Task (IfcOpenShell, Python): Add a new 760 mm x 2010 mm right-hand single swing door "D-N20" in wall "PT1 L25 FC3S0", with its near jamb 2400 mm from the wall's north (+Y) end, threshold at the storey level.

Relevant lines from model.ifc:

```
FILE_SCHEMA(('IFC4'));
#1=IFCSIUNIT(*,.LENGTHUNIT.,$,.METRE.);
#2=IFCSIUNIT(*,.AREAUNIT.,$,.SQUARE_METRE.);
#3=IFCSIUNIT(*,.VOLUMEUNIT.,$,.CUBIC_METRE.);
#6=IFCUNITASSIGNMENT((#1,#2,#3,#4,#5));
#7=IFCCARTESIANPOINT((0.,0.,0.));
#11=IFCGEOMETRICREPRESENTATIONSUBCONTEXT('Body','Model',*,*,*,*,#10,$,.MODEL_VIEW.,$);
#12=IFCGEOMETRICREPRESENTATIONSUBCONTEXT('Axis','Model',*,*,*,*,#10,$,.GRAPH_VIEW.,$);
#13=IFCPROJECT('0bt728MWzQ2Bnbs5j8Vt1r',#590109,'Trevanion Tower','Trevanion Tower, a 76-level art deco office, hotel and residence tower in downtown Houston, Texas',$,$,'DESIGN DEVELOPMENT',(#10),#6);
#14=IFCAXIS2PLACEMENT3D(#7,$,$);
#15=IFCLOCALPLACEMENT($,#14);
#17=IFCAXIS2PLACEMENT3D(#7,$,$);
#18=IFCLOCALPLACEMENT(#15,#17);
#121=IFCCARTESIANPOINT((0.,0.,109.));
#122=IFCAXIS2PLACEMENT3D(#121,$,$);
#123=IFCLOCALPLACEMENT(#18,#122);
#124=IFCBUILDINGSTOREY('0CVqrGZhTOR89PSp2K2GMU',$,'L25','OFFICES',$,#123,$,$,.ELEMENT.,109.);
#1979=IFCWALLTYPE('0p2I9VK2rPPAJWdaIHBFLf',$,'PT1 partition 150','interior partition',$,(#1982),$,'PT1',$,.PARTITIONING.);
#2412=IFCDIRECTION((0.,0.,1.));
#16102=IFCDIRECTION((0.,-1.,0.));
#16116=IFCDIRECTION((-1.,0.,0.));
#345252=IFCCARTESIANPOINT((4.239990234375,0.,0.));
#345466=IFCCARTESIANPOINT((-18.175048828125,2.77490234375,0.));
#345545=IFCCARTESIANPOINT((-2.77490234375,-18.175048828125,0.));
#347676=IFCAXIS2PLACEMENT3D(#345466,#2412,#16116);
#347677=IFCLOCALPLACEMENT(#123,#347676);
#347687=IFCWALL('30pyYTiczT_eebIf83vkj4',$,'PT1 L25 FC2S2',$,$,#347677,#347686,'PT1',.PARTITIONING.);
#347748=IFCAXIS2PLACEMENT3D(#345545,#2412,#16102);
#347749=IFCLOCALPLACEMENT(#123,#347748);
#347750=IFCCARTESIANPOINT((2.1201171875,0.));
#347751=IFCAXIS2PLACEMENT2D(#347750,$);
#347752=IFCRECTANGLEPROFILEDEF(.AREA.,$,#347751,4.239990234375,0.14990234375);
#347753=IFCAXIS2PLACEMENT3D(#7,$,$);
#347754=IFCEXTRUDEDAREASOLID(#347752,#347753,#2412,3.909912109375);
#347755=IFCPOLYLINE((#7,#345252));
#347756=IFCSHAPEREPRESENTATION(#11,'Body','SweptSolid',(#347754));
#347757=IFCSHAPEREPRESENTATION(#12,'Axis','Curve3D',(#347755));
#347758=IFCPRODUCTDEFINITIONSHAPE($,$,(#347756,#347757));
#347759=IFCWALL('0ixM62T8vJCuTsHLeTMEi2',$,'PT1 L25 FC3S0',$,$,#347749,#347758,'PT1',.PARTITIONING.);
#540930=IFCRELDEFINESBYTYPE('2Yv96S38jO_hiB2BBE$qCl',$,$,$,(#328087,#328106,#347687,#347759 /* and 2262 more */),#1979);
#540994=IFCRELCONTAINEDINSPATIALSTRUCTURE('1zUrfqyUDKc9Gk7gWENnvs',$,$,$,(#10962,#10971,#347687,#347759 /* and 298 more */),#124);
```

```python
import numpy as np
import ifcopenshell
import ifcopenshell.api.feature
import ifcopenshell.api.geometry
import ifcopenshell.api.root
import ifcopenshell.api.spatial
import ifcopenshell.geom
import ifcopenshell.util.element
import ifcopenshell.util.placement
import ifcopenshell.util.representation
import ifcopenshell.util.shape
import ifcopenshell.util.unit

model = ifcopenshell.open("model.ifc")
unit_scale = ifcopenshell.util.unit.calculate_unit_scale(model)
settings = ifcopenshell.geom.settings()


def volume(element):
    """Net volume in cubic metres, openings subtracted."""
    shape = ifcopenshell.geom.create_shape(settings, element)
    return ifcopenshell.util.shape.get_volume(shape.geometry)


wall = model.by_guid("0ixM62T8vJCuTsHLeTMEi2")
storey = ifcopenshell.util.element.get_container(wall, ifc_class="IfcBuildingStorey")
context = ifcopenshell.util.representation.get_context(model, "Model", "Body", "MODEL_VIEW")
before = volume(wall)

width, height, from_end, sill = 0.76, 2.01, 2.4, 0.0  # metres

# The wall runs along its own X axis, and the end named is its -X end.
wall_shape = ifcopenshell.geom.create_shape(settings, wall)
x, y, z = ifcopenshell.util.shape.get_vertices(wall_shape.geometry).T
start = x.min() + from_end
face, thickness = float(y.min()), float(y.max() - y.min())
wall_matrix = ifcopenshell.util.placement.get_local_placement(wall.ObjectPlacement)
level = ifcopenshell.util.placement.get_local_placement(storey.ObjectPlacement)[2, 3]


def in_wall(x, y):
    """Placement at x, y metres in the wall's axes, at sill height."""
    matrix = wall_matrix.copy()
    matrix[:, 3] = wall_matrix @ np.array([x / unit_scale, y / unit_scale, 0.0, 1.0])
    matrix[2, 3] = level + sill / unit_scale
    return matrix


# Opening: a box that overshoots both wall faces by 50 mm.
opening = ifcopenshell.api.root.create_entity(model, ifc_class="IfcOpeningElement", predefined_type="OPENING")
box = ifcopenshell.api.geometry.add_wall_representation(
    model, context=context, length=width, height=height, thickness=thickness + 0.1
)
ifcopenshell.api.geometry.assign_representation(model, product=opening, representation=box)
ifcopenshell.api.geometry.edit_object_placement(model, product=opening, matrix=in_wall(start, face - 0.05), is_si=False)
ifcopenshell.api.feature.add_feature(model, feature=opening, element=wall)

door = ifcopenshell.api.root.create_entity(model, ifc_class="IfcDoor", name="D-N20", predefined_type="DOOR")
door.OverallWidth, door.OverallHeight = width / unit_scale, height / unit_scale
door.OperationType = "SINGLE_SWING_RIGHT"
body = ifcopenshell.api.geometry.add_door_representation(
    model,
    context=context,
    overall_width=door.OverallWidth,
    overall_height=door.OverallHeight,
    operation_type="SINGLE_SWING_RIGHT",
    lining_properties={"LiningDepth": thickness / unit_scale, "ThresholdDepth": thickness / unit_scale},
)
ifcopenshell.api.geometry.assign_representation(model, product=door, representation=body)
ifcopenshell.api.spatial.assign_container(model, products=[door], relating_structure=storey)
ifcopenshell.api.feature.add_filling(model, opening=opening, element=door)

# The lining spans the wall, so the door starts at the wall face.
ifcopenshell.api.geometry.edit_object_placement(model, product=door, matrix=in_wall(start, face), is_si=False)

after = volume(wall)

print(f"wall volume {before:.3f} -> {after:.3f} m3")

model.write("model_edited.ifc")
```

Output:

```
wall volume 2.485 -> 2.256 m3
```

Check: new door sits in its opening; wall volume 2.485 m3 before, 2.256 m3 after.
